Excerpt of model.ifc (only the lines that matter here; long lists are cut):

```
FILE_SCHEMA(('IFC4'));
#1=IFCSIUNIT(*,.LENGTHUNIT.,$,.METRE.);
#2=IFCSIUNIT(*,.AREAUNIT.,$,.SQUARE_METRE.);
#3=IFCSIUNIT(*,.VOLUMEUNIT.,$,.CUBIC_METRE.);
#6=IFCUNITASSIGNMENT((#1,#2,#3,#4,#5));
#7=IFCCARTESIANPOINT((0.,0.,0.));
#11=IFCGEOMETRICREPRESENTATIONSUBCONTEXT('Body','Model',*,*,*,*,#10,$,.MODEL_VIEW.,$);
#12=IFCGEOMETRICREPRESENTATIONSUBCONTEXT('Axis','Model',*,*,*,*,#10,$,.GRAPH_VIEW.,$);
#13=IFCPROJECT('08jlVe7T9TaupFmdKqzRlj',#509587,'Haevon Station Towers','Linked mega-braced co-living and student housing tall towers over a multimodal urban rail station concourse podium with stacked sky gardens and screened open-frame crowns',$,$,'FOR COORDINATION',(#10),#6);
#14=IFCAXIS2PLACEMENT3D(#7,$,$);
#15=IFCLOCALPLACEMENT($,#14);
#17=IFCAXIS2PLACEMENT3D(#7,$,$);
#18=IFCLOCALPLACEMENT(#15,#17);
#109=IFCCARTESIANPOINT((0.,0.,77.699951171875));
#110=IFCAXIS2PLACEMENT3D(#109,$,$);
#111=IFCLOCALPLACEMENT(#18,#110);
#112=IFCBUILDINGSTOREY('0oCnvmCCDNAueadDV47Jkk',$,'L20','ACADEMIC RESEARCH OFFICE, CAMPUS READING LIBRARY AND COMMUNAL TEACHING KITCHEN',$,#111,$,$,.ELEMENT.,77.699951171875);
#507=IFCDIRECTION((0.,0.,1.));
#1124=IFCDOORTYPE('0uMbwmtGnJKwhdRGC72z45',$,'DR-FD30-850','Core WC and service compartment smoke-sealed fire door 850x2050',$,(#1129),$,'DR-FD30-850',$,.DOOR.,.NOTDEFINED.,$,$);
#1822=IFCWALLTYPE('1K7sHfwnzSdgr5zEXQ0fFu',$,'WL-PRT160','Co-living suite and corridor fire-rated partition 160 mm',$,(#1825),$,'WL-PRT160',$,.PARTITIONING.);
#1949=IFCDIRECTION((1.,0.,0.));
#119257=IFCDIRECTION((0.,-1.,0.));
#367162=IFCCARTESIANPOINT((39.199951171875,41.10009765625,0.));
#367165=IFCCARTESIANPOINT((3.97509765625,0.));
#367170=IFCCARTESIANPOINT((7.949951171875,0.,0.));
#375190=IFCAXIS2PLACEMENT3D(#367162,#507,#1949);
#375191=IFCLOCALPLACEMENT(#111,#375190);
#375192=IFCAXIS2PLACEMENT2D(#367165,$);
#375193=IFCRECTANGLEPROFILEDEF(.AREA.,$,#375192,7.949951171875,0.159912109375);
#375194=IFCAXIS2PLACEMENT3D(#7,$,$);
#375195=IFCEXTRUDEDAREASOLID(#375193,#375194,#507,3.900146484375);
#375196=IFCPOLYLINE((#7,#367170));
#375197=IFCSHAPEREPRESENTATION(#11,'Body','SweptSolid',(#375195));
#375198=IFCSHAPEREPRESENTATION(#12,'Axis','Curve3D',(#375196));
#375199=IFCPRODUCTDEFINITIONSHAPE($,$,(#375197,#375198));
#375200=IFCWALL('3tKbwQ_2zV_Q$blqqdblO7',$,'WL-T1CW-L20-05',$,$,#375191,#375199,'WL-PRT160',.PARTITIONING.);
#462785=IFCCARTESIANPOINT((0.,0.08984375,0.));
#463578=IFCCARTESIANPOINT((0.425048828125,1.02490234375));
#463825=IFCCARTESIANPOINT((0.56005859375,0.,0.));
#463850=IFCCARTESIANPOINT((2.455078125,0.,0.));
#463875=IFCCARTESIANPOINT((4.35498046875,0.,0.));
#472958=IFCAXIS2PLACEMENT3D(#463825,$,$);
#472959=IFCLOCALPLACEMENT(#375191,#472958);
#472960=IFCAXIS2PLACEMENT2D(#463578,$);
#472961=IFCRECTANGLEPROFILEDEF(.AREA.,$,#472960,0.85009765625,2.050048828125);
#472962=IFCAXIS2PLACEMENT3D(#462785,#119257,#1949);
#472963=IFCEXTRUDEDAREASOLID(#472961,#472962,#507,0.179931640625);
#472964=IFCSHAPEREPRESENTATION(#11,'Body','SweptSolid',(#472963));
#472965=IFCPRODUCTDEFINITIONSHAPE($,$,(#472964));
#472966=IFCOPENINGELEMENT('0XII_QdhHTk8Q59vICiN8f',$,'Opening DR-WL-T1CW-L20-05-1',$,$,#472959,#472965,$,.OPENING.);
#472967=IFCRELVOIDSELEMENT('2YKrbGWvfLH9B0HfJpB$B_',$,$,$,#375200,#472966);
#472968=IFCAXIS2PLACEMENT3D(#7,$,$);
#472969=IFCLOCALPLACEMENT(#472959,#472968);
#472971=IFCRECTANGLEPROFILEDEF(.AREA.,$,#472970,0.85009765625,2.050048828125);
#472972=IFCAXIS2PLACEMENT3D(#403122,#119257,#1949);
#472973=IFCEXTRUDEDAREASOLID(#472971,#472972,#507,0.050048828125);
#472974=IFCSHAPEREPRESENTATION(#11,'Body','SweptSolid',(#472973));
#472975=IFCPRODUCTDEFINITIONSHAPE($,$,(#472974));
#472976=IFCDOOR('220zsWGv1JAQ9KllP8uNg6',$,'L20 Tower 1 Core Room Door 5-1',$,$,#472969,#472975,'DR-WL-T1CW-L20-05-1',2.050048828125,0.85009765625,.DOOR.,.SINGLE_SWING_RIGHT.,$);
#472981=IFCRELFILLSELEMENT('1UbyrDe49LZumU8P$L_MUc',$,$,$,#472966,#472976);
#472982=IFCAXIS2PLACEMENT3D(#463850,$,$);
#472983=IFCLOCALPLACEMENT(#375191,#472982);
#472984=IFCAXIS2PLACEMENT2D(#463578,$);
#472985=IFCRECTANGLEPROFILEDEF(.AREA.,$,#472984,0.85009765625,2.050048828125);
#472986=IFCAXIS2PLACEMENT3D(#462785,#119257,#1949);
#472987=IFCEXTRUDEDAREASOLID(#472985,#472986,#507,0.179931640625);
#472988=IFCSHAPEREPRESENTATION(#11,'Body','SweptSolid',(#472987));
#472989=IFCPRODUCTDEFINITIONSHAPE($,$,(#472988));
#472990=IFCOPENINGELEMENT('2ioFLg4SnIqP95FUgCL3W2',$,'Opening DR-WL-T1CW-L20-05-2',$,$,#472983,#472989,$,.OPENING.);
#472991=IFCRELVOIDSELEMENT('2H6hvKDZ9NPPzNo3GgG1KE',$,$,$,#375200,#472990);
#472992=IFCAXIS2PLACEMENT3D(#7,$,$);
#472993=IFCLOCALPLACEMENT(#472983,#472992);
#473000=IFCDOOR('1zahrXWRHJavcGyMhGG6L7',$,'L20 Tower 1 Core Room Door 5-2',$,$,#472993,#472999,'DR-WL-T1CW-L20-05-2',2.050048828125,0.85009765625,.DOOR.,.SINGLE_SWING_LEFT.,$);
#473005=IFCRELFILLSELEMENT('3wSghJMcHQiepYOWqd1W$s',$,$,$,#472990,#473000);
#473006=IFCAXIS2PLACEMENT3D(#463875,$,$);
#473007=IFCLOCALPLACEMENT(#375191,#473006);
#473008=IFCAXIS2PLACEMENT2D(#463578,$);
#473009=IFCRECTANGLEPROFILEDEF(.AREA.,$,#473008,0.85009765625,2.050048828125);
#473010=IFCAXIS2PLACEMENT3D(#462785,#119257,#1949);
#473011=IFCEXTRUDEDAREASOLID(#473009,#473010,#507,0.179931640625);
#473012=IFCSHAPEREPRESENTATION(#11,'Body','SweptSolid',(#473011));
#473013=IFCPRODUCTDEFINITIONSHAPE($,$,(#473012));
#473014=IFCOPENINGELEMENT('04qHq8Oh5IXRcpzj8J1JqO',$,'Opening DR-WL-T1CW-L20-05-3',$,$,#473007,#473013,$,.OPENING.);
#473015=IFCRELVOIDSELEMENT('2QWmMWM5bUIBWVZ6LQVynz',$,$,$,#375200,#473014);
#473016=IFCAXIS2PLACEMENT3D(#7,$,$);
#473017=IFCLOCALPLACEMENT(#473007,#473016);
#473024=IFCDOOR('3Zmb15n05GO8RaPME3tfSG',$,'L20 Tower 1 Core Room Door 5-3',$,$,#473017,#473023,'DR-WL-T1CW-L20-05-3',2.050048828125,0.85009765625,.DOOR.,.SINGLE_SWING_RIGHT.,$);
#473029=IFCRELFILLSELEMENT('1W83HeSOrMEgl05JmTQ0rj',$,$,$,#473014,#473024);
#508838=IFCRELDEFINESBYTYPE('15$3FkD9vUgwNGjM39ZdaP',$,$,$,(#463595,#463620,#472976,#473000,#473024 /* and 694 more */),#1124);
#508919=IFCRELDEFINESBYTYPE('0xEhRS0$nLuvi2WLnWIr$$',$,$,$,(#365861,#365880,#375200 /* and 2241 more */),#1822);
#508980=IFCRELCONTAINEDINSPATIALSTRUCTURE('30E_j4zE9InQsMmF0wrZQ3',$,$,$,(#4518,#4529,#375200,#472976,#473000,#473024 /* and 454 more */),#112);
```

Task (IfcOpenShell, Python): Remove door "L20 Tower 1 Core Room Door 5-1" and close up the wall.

```python
import ifcopenshell
import ifcopenshell.api.feature
import ifcopenshell.api.root
import ifcopenshell.geom
import ifcopenshell.util.shape

model = ifcopenshell.open("model.ifc")
settings = ifcopenshell.geom.settings()


def volume(element):
    """Net volume in cubic metres, openings subtracted."""
    shape = ifcopenshell.geom.create_shape(settings, element)
    return ifcopenshell.util.shape.get_volume(shape.geometry)


door = model.by_guid("220zsWGv1JAQ9KllP8uNg6")
opening = door.FillsVoids[0].RelatingOpeningElement
wall = opening.VoidsElements[0].RelatingBuildingElement
before = volume(wall)

ifcopenshell.api.root.remove_product(model, product=door)
ifcopenshell.api.feature.remove_feature(model, feature=opening)

after = volume(wall)

print(f"wall volume {before:.3f} -> {after:.3f} m3")

model.write("model-out.ifc")
```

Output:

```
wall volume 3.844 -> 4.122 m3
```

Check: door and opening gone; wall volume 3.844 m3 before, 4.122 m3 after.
